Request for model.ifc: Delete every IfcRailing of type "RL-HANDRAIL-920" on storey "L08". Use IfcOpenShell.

First a look at what the model holds.

```python
import ifcopenshell
import ifcopenshell.util.element

model = ifcopenshell.open("model.ifc")
print(model.schema)
storey = next(s for s in model.by_type("IfcBuildingStorey") if s.Name == "L08")
railings = [e for e in ifcopenshell.util.element.get_decomposition(storey) if e.is_a("IfcRailing")]
seen = {}
for e in railings:
    element_type = ifcopenshell.util.element.get_type(e)
    name = element_type.Name if element_type not in (None, e) else None
    seen[name] = seen.get(name, 0) + 1
for name, count in sorted(seen.items(), key=str):
    print(count, "x", name)
```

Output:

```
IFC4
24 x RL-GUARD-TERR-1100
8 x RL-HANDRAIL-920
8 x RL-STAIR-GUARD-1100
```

```python
import ifcopenshell
import ifcopenshell.api.root
import ifcopenshell.util.element

model = ifcopenshell.open("model.ifc")

storey = next(s for s in model.by_type("IfcBuildingStorey") if s.Name == "L08")
railings = [e for e in ifcopenshell.util.element.get_decomposition(storey) if e.is_a("IfcRailing")]
targets = [e for e in railings if (t := ifcopenshell.util.element.get_type(e)) not in (None, e) and t.Name == "RL-HANDRAIL-920"]

for e in targets:
    ifcopenshell.api.root.remove_product(model, product=e)
print(len(targets), "removed")

model.write("model_v2.ifc")
```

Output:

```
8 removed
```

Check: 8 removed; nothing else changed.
